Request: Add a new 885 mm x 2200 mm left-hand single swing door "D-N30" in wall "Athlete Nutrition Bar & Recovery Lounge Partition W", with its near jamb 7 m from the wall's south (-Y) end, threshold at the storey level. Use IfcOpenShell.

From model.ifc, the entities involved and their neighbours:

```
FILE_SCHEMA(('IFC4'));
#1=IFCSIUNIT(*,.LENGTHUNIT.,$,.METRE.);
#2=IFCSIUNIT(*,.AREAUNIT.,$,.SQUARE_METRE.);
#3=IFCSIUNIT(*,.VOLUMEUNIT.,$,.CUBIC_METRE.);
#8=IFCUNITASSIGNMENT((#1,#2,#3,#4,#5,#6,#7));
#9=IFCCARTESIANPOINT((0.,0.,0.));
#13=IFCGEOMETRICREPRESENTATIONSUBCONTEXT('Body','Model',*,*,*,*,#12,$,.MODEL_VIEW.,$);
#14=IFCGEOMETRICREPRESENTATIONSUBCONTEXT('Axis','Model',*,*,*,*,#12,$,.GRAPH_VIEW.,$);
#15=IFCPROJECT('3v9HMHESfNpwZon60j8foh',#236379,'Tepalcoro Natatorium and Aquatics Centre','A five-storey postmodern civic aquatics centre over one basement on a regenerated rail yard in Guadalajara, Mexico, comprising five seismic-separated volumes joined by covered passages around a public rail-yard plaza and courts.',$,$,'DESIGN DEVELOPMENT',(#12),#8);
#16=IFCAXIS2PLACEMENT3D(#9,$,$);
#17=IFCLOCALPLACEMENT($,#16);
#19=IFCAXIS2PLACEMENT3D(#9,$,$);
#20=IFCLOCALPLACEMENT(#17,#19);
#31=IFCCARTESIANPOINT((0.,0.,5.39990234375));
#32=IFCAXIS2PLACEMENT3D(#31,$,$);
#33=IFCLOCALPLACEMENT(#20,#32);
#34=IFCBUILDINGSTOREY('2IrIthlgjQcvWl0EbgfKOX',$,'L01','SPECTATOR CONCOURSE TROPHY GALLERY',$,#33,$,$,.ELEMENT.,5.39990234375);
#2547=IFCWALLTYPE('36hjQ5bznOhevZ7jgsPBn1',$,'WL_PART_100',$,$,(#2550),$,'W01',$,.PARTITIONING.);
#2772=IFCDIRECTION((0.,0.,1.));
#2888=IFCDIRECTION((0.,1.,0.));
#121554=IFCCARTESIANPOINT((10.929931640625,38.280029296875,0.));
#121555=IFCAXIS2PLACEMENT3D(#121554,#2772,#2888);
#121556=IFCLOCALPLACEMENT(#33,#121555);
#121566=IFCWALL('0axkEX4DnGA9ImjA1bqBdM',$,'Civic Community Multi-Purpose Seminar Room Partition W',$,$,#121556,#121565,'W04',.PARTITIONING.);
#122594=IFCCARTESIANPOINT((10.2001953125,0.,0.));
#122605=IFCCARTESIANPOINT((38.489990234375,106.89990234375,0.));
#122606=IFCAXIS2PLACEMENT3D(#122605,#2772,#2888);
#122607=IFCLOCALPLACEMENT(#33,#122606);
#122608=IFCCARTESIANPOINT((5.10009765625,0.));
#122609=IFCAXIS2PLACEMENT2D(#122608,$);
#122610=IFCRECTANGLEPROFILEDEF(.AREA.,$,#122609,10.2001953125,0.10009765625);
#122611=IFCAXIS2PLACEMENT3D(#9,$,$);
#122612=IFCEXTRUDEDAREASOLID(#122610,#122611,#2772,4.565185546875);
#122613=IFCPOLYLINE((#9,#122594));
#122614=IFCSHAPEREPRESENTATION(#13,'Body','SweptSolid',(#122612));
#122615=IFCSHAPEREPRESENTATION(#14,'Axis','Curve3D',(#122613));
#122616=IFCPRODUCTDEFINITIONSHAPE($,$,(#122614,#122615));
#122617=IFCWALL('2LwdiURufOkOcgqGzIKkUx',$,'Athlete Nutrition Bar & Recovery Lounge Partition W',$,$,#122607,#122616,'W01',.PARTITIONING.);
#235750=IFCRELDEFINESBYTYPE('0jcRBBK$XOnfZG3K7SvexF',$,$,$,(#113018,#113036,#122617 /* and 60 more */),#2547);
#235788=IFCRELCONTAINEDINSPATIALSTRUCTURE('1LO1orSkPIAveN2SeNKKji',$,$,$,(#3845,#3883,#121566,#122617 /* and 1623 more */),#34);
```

```python
import numpy as np
import ifcopenshell
import ifcopenshell.api.feature
import ifcopenshell.api.geometry
import ifcopenshell.api.root
import ifcopenshell.api.spatial
import ifcopenshell.geom
import ifcopenshell.util.element
import ifcopenshell.util.placement
import ifcopenshell.util.representation
import ifcopenshell.util.shape
import ifcopenshell.util.unit

model = ifcopenshell.open("model.ifc")
unit_scale = ifcopenshell.util.unit.calculate_unit_scale(model)
settings = ifcopenshell.geom.settings()


def volume(element):
    """Net volume in cubic metres, openings subtracted."""
    shape = ifcopenshell.geom.create_shape(settings, element)
    return ifcopenshell.util.shape.get_volume(shape.geometry)


wall = model.by_id(122617)
storey = ifcopenshell.util.element.get_container(wall, ifc_class="IfcBuildingStorey")
context = ifcopenshell.util.representation.get_context(model, "Model", "Body", "MODEL_VIEW")
before = volume(wall)

width, height, from_end, sill = 0.885, 2.2, 7, 0.0  # metres

# The wall runs along its own X axis, and the end named is its -X end.
wall_shape = ifcopenshell.geom.create_shape(settings, wall)
x, y, z = ifcopenshell.util.shape.get_vertices(wall_shape.geometry).T
start = x.min() + from_end
face, thickness = float(y.min()), float(y.max() - y.min())
wall_matrix = ifcopenshell.util.placement.get_local_placement(wall.ObjectPlacement)
level = ifcopenshell.util.placement.get_local_placement(storey.ObjectPlacement)[2, 3]


def in_wall(x, y):
    """Placement at x, y metres in the wall's axes, at sill height."""
    matrix = wall_matrix.copy()
    matrix[:, 3] = wall_matrix @ np.array([x / unit_scale, y / unit_scale, 0.0, 1.0])
    matrix[2, 3] = level + sill / unit_scale
    return matrix


# Opening: a box that overshoots both wall faces by 50 mm.
opening = ifcopenshell.api.root.create_entity(model, ifc_class="IfcOpeningElement", predefined_type="OPENING")
box = ifcopenshell.api.geometry.add_wall_representation(
    model, context=context, length=width, height=height, thickness=thickness + 0.1
)
ifcopenshell.api.geometry.assign_representation(model, product=opening, representation=box)
ifcopenshell.api.geometry.edit_object_placement(model, product=opening, matrix=in_wall(start, face - 0.05), is_si=False)
ifcopenshell.api.feature.add_feature(model, feature=opening, element=wall)

door = ifcopenshell.api.root.create_entity(model, ifc_class="IfcDoor", name="D-N30", predefined_type="DOOR")
door.OverallWidth, door.OverallHeight = width / unit_scale, height / unit_scale
door.OperationType = "SINGLE_SWING_LEFT"
body = ifcopenshell.api.geometry.add_door_representation(
    model,
    context=context,
    overall_width=door.OverallWidth,
    overall_height=door.OverallHeight,
    operation_type="SINGLE_SWING_LEFT",
    lining_properties={"LiningDepth": thickness / unit_scale, "ThresholdDepth": thickness / unit_scale},
)
ifcopenshell.api.geometry.assign_representation(model, product=door, representation=body)
ifcopenshell.api.spatial.assign_container(model, products=[door], relating_structure=storey)
ifcopenshell.api.feature.add_filling(model, opening=opening, element=door)

# The lining spans the wall, so the door starts at the wall face.
ifcopenshell.api.geometry.edit_object_placement(model, product=door, matrix=in_wall(start, face), is_si=False)

after = volume(wall)

print(f"wall volume {before:.3f} -> {after:.3f} m3")

model.write("model_updated.ifc")
```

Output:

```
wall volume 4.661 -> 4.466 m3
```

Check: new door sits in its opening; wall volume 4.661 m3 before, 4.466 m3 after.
